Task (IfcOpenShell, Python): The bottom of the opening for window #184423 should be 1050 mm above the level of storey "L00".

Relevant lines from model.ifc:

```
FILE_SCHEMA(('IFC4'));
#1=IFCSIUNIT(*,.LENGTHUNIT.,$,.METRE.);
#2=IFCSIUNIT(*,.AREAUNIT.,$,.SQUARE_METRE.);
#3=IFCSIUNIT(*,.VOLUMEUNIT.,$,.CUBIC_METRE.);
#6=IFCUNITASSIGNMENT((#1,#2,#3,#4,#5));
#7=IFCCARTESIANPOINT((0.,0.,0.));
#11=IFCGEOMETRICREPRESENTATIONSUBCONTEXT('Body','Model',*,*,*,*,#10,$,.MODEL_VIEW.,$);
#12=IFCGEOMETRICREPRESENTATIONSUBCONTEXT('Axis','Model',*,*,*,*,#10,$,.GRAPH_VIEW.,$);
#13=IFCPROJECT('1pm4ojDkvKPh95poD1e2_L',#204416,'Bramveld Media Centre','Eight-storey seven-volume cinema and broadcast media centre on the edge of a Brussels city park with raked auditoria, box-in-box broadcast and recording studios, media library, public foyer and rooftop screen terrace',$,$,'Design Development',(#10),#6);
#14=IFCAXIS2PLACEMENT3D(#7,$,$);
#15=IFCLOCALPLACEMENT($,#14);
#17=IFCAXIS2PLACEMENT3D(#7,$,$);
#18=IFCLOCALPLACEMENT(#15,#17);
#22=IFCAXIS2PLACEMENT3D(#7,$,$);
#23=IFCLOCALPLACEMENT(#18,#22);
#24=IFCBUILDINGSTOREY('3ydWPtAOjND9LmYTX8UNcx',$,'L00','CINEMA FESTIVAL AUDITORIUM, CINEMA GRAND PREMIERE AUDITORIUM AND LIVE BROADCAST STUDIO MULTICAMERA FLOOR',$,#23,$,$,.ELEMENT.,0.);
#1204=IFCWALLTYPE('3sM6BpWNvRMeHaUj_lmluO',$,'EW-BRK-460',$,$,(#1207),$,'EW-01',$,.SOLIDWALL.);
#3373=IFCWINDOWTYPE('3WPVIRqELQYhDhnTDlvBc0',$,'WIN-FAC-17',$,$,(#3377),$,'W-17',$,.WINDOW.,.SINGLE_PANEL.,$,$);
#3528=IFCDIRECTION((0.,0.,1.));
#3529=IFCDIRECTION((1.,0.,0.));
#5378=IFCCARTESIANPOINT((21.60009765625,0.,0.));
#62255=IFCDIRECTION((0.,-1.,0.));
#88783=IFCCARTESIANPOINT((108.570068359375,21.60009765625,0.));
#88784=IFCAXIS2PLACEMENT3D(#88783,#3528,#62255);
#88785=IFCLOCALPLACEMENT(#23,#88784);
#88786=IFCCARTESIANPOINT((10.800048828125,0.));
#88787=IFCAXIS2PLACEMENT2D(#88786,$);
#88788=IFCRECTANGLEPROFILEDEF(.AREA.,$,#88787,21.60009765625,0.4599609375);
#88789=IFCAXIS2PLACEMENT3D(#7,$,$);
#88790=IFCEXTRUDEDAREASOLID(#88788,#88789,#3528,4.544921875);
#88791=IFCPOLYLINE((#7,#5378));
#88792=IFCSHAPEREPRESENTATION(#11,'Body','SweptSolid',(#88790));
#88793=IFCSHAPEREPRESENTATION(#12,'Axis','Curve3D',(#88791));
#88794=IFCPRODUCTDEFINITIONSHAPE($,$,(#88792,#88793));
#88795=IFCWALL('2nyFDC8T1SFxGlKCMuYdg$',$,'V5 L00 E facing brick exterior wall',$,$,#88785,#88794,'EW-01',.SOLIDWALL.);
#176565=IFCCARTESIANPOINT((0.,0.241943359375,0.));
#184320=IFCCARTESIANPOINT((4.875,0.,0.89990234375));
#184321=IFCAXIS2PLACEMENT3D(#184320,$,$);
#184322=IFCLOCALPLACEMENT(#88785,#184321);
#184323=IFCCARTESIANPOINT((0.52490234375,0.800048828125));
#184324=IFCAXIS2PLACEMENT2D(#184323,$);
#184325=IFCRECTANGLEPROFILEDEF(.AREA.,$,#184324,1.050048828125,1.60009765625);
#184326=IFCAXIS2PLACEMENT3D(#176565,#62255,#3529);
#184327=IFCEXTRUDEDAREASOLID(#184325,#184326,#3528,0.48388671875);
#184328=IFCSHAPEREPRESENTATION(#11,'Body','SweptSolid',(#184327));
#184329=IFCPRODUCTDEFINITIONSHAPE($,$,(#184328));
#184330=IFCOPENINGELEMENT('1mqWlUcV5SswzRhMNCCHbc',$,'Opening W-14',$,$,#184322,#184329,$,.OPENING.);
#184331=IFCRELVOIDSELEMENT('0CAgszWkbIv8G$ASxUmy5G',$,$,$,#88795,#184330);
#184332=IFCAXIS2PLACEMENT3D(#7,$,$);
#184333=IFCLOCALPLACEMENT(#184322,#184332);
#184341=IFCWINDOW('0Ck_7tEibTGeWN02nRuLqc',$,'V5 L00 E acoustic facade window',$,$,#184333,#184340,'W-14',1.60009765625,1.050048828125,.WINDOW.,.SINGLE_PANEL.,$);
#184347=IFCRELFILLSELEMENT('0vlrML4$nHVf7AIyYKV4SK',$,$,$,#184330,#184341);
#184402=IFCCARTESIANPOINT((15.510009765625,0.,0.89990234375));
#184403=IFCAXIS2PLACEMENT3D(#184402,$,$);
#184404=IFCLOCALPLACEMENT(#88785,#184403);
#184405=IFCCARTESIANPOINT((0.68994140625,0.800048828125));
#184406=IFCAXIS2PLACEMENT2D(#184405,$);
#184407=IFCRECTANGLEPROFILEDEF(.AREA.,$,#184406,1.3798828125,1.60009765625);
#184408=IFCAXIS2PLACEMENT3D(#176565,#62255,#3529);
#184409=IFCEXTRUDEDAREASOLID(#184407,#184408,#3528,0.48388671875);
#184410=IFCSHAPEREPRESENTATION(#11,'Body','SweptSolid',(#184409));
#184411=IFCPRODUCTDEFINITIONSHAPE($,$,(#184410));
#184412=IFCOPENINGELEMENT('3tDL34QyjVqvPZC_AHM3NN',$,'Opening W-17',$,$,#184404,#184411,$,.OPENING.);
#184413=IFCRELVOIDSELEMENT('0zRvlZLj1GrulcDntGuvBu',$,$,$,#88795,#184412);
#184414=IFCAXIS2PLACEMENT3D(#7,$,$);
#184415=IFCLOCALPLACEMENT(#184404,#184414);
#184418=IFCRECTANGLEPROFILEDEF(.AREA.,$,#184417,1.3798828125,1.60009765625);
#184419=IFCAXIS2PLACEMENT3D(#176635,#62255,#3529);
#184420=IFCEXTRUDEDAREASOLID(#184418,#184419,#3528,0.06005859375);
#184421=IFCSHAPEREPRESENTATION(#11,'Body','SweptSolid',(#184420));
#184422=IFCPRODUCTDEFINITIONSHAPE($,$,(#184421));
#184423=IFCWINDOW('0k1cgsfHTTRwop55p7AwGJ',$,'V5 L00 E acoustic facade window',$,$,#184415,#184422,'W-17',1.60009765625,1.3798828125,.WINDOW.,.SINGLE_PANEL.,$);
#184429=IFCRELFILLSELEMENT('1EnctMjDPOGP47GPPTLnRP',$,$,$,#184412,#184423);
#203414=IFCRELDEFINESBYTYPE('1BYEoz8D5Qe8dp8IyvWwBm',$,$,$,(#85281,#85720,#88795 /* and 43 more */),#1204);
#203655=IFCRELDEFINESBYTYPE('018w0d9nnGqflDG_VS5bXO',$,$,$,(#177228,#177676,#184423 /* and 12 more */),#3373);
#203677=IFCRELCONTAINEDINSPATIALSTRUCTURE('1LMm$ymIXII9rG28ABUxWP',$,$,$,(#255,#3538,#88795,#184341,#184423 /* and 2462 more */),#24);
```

```python
import numpy as np
import ifcopenshell
import ifcopenshell.api.geometry
import ifcopenshell.geom
import ifcopenshell.util.element
import ifcopenshell.util.placement
import ifcopenshell.util.shape
import ifcopenshell.util.unit

model = ifcopenshell.open("model.ifc")
unit_scale = ifcopenshell.util.unit.calculate_unit_scale(model)

window = model.by_id(184423)
opening = window.FillsVoids[0].RelatingOpeningElement
storey = ifcopenshell.util.element.get_container(window, ifc_class="IfcBuildingStorey")
level = ifcopenshell.util.placement.get_local_placement(storey.ObjectPlacement)[2, 3]

# The opening's origin need not be at the sill, so measure its lowest point.
shape = ifcopenshell.geom.create_shape(ifcopenshell.geom.settings(), opening)
bottom = ifcopenshell.util.shape.get_shape_bottom_elevation(shape, shape.geometry) / unit_scale
dz = level + 1.05 / unit_scale - bottom

shift = np.array([0.0, 0.0, dz])
# The window is placed relative to its opening, so it follows when the opening moves.
matrix = ifcopenshell.util.placement.get_local_placement(opening.ObjectPlacement)
matrix[:3, 3] += shift
ifcopenshell.api.geometry.edit_object_placement(
    model, product=opening, matrix=matrix, is_si=False, should_transform_children=True
)

print(f"moved by {dz * unit_scale:+.3f} m")

model.write("model_updated.ifc")
```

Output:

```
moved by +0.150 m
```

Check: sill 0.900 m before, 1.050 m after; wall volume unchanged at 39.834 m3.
